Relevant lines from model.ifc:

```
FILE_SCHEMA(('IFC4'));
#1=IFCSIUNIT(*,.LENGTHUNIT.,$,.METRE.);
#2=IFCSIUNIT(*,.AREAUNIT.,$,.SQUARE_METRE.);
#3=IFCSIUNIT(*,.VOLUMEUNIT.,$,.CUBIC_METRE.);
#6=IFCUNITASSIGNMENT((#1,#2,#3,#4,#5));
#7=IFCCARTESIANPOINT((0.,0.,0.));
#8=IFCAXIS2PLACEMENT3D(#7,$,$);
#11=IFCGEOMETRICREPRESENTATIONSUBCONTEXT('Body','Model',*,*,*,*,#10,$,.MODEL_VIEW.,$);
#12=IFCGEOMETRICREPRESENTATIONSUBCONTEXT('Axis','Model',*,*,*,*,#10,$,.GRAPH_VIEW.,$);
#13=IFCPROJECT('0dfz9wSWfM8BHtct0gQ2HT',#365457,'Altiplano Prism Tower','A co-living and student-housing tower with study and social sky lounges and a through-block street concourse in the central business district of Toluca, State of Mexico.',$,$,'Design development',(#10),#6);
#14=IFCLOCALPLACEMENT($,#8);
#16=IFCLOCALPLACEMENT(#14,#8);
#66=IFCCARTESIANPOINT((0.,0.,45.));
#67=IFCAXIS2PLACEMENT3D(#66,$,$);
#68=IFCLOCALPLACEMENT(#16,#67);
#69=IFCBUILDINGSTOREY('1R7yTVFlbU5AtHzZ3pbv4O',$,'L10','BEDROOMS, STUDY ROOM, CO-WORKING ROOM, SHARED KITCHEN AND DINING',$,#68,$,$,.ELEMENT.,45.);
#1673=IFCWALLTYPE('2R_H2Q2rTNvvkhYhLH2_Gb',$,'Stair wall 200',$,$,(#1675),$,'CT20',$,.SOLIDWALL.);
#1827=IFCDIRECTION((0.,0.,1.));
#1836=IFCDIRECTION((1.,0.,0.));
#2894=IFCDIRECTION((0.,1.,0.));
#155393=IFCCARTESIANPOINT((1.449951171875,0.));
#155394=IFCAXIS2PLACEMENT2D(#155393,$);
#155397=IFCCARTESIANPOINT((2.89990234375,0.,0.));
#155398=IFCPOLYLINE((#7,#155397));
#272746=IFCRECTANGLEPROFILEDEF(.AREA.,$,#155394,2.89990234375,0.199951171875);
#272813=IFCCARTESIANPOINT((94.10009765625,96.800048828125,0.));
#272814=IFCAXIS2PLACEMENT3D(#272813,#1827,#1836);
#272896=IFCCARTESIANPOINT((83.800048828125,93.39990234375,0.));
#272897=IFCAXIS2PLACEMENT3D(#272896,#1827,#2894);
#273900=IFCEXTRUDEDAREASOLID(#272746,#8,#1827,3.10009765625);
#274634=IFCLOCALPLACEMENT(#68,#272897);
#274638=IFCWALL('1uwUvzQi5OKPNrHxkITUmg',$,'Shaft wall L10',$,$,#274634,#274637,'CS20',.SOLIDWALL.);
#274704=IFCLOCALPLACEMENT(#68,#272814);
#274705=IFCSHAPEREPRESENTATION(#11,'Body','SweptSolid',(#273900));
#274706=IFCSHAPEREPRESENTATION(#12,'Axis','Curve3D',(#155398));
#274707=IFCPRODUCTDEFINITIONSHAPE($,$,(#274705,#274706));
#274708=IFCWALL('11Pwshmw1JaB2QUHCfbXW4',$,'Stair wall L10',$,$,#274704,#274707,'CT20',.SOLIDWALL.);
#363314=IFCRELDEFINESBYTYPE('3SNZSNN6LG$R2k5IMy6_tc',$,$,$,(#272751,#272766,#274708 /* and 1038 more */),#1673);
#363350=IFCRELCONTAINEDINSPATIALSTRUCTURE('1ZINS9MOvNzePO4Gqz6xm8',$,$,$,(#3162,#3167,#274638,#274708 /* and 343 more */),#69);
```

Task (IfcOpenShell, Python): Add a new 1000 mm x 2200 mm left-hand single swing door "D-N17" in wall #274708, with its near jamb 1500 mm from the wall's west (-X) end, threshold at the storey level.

```python
import numpy as np
import ifcopenshell
import ifcopenshell.api.feature
import ifcopenshell.api.geometry
import ifcopenshell.api.root
import ifcopenshell.api.spatial
import ifcopenshell.geom
import ifcopenshell.util.element
import ifcopenshell.util.placement
import ifcopenshell.util.representation
import ifcopenshell.util.shape
import ifcopenshell.util.unit

model = ifcopenshell.open("model.ifc")
unit_scale = ifcopenshell.util.unit.calculate_unit_scale(model)
settings = ifcopenshell.geom.settings()


def volume(element):
    """Net volume in cubic metres, openings subtracted."""
    shape = ifcopenshell.geom.create_shape(settings, element)
    return ifcopenshell.util.shape.get_volume(shape.geometry)


wall = model.by_guid("11Pwshmw1JaB2QUHCfbXW4")
storey = ifcopenshell.util.element.get_container(wall, ifc_class="IfcBuildingStorey")
context = ifcopenshell.util.representation.get_context(model, "Model", "Body", "MODEL_VIEW")
before = volume(wall)

width, height, from_end, sill = 1, 2.2, 1.5, 0.0  # metres

# The wall runs along its own X axis, and the end named is its -X end.
wall_shape = ifcopenshell.geom.create_shape(settings, wall)
x, y, z = ifcopenshell.util.shape.get_vertices(wall_shape.geometry).T
start = x.min() + from_end
face, thickness = float(y.min()), float(y.max() - y.min())
wall_matrix = ifcopenshell.util.placement.get_local_placement(wall.ObjectPlacement)
level = ifcopenshell.util.placement.get_local_placement(storey.ObjectPlacement)[2, 3]


def in_wall(x, y):
    """Placement at x, y metres in the wall's axes, at sill height."""
    matrix = wall_matrix.copy()
    matrix[:, 3] = wall_matrix @ np.array([x / unit_scale, y / unit_scale, 0.0, 1.0])
    matrix[2, 3] = level + sill / unit_scale
    return matrix


# Opening: a box that overshoots both wall faces by 50 mm.
opening = ifcopenshell.api.root.create_entity(model, ifc_class="IfcOpeningElement", predefined_type="OPENING")
box = ifcopenshell.api.geometry.add_wall_representation(
    model, context=context, length=width, height=height, thickness=thickness + 0.1
)
ifcopenshell.api.geometry.assign_representation(model, product=opening, representation=box)
ifcopenshell.api.geometry.edit_object_placement(model, product=opening, matrix=in_wall(start, face - 0.05), is_si=False)
ifcopenshell.api.feature.add_feature(model, feature=opening, element=wall)

door = ifcopenshell.api.root.create_entity(model, ifc_class="IfcDoor", name="D-N17", predefined_type="DOOR")
door.OverallWidth, door.OverallHeight = width / unit_scale, height / unit_scale
door.OperationType = "SINGLE_SWING_LEFT"
body = ifcopenshell.api.geometry.add_door_representation(
    model,
    context=context,
    overall_width=door.OverallWidth,
    overall_height=door.OverallHeight,
    operation_type="SINGLE_SWING_LEFT",
    lining_properties={"LiningDepth": thickness / unit_scale, "ThresholdDepth": thickness / unit_scale},
)
ifcopenshell.api.geometry.assign_representation(model, product=door, representation=body)
ifcopenshell.api.spatial.assign_container(model, products=[door], relating_structure=storey)
ifcopenshell.api.feature.add_filling(model, opening=opening, element=door)

# The lining spans the wall, so the door starts at the wall face.
ifcopenshell.api.geometry.edit_object_placement(model, product=door, matrix=in_wall(start, face), is_si=False)

after = volume(wall)

print(f"wall volume {before:.3f} -> {after:.3f} m3")

model.write("model_updated.ifc")
```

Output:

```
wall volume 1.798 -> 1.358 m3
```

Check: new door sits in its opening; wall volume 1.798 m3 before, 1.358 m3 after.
